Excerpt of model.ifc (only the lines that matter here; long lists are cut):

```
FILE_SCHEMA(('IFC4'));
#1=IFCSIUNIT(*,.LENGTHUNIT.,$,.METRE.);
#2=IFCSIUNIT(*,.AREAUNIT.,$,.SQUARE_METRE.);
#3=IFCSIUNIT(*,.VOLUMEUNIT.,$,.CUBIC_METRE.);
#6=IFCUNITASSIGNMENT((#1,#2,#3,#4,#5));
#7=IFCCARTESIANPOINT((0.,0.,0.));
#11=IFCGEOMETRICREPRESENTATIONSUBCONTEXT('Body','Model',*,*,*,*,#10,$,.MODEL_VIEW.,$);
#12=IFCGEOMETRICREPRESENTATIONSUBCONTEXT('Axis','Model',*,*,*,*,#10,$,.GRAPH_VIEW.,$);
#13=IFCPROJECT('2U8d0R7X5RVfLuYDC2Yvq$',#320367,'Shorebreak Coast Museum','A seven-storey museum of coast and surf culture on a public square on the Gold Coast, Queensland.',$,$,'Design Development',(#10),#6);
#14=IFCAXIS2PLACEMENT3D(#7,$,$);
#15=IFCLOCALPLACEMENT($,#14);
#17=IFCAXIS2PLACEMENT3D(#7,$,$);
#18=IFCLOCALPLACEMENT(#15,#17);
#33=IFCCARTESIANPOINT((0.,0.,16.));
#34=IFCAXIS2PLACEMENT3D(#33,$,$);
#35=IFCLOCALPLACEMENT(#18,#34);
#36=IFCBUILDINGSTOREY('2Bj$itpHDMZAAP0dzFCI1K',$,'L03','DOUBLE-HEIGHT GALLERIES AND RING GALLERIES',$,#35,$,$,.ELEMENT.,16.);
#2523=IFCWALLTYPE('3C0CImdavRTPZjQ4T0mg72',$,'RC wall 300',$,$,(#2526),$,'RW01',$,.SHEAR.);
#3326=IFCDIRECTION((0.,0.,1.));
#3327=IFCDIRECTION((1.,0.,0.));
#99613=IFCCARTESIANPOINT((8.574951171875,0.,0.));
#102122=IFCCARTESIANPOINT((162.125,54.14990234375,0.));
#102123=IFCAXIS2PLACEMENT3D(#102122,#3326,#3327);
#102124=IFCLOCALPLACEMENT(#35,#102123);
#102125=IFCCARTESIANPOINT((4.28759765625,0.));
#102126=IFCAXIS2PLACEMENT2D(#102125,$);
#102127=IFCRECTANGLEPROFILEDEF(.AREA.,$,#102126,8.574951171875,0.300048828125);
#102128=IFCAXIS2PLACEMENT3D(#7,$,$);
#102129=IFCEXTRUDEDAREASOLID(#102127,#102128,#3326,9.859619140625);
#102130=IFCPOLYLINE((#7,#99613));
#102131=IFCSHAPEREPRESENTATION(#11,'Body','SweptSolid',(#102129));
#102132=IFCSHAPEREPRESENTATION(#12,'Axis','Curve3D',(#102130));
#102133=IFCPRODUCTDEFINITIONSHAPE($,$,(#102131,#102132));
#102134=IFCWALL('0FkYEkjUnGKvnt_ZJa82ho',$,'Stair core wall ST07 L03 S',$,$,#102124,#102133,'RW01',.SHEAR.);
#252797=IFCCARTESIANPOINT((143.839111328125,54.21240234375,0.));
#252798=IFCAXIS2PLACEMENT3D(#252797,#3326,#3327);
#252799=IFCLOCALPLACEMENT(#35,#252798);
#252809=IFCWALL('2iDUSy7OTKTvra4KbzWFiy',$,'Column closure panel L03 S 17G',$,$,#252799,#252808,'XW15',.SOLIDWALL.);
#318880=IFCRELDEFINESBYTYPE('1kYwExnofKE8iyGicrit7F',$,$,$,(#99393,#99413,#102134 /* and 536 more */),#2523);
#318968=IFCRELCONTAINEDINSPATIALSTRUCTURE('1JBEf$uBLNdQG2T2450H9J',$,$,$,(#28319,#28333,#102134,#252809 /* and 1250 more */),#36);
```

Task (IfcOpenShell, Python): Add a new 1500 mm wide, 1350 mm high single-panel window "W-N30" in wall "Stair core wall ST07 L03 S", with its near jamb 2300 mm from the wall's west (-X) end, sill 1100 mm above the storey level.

```python
import numpy as np
import ifcopenshell
import ifcopenshell.api.feature
import ifcopenshell.api.geometry
import ifcopenshell.api.root
import ifcopenshell.api.spatial
import ifcopenshell.geom
import ifcopenshell.util.element
import ifcopenshell.util.placement
import ifcopenshell.util.representation
import ifcopenshell.util.shape
import ifcopenshell.util.unit

model = ifcopenshell.open("model.ifc")
unit_scale = ifcopenshell.util.unit.calculate_unit_scale(model)
settings = ifcopenshell.geom.settings()


def volume(element):
    """Net volume in cubic metres, openings subtracted."""
    shape = ifcopenshell.geom.create_shape(settings, element)
    return ifcopenshell.util.shape.get_volume(shape.geometry)


wall = model.by_id(102134)
storey = ifcopenshell.util.element.get_container(wall, ifc_class="IfcBuildingStorey")
context = ifcopenshell.util.representation.get_context(model, "Model", "Body", "MODEL_VIEW")
before = volume(wall)

width, height, from_end, sill = 1.5, 1.35, 2.3, 1.1  # metres

# The wall runs along its own X axis, and the end named is its -X end.
wall_shape = ifcopenshell.geom.create_shape(settings, wall)
x, y, z = ifcopenshell.util.shape.get_vertices(wall_shape.geometry).T
start = x.min() + from_end
face, thickness = float(y.min()), float(y.max() - y.min())
wall_matrix = ifcopenshell.util.placement.get_local_placement(wall.ObjectPlacement)
level = ifcopenshell.util.placement.get_local_placement(storey.ObjectPlacement)[2, 3]


def in_wall(x, y):
    """Placement at x, y metres in the wall's axes, at sill height."""
    matrix = wall_matrix.copy()
    matrix[:, 3] = wall_matrix @ np.array([x / unit_scale, y / unit_scale, 0.0, 1.0])
    matrix[2, 3] = level + sill / unit_scale
    return matrix


# Opening: a box that overshoots both wall faces by 50 mm.
opening = ifcopenshell.api.root.create_entity(model, ifc_class="IfcOpeningElement", predefined_type="OPENING")
box = ifcopenshell.api.geometry.add_wall_representation(
    model, context=context, length=width, height=height, thickness=thickness + 0.1
)
ifcopenshell.api.geometry.assign_representation(model, product=opening, representation=box)
ifcopenshell.api.geometry.edit_object_placement(model, product=opening, matrix=in_wall(start, face - 0.05), is_si=False)
ifcopenshell.api.feature.add_feature(model, feature=opening, element=wall)

window = ifcopenshell.api.root.create_entity(model, ifc_class="IfcWindow", name="W-N30", predefined_type="WINDOW")
window.OverallWidth, window.OverallHeight = width / unit_scale, height / unit_scale
window.PartitioningType = "SINGLE_PANEL"
body = ifcopenshell.api.geometry.add_window_representation(
    model,
    context=context,
    overall_width=window.OverallWidth,
    overall_height=window.OverallHeight,
    partition_type="SINGLE_PANEL",
)
ifcopenshell.api.geometry.assign_representation(model, product=window, representation=body)
ifcopenshell.api.spatial.assign_container(model, products=[window], relating_structure=storey)
ifcopenshell.api.feature.add_filling(model, opening=opening, element=window)

# Centre the window in the wall's thickness.
ifcopenshell.api.geometry.edit_object_placement(model, product=window, matrix=in_wall(start, face), is_si=False)
window_shape = ifcopenshell.geom.create_shape(settings, window)
depth = ifcopenshell.util.shape.get_vertices(window_shape.geometry)[:, 1]
offset = face + thickness / 2 - (depth.min() + depth.max()) / 2
ifcopenshell.api.geometry.edit_object_placement(model, product=window, matrix=in_wall(start, offset), is_si=False)

after = volume(wall)

print(f"wall volume {before:.3f} -> {after:.3f} m3")

model.write("model_rev.ifc")
```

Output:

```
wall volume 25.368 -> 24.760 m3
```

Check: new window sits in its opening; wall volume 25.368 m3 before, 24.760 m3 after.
